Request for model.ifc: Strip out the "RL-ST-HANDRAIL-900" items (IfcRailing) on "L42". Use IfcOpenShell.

First a look at what the model holds.

```python
import ifcopenshell
import ifcopenshell.util.element

model = ifcopenshell.open("model.ifc")
print(model.schema)
storey = next(s for s in model.by_type("IfcBuildingStorey") if s.Name == "L42")
railings = [e for e in ifcopenshell.util.element.get_decomposition(storey) if e.is_a("IfcRailing")]
seen = {}
for e in railings:
    element_type = ifcopenshell.util.element.get_type(e)
    name = element_type.Name if element_type not in (None, e) else None
    seen[name] = seen.get(name, 0) + 1
for name, count in sorted(seen.items(), key=str):
    print(count, "x", name)
```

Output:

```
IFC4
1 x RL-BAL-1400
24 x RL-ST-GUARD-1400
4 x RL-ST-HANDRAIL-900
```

```python
import ifcopenshell
import ifcopenshell.api.root
import ifcopenshell.util.element

model = ifcopenshell.open("model.ifc")

storey = next(s for s in model.by_type("IfcBuildingStorey") if s.Name == "L42")
railings = [e for e in ifcopenshell.util.element.get_decomposition(storey) if e.is_a("IfcRailing")]
targets = [e for e in railings if (t := ifcopenshell.util.element.get_type(e)) not in (None, e) and t.Name == "RL-ST-HANDRAIL-900"]

for e in targets:
    ifcopenshell.api.root.remove_product(model, product=e)
print(len(targets), "removed")

model.write("model_edited.ifc")
```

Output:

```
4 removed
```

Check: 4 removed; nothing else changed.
